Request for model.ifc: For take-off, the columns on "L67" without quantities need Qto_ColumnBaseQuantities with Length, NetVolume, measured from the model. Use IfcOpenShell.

First a look at what the model holds.

```python
import ifcopenshell
import ifcopenshell.util.element
import ifcopenshell.util.unit

model = ifcopenshell.open("model.ifc")
print(model.schema)
for unit_type in ("LENGTHUNIT", "AREAUNIT", "VOLUMEUNIT"):
    print(unit_type, ifcopenshell.util.unit.calculate_unit_scale(model, unit_type))
storey = next(s for s in model.by_type("IfcBuildingStorey") if s.Name == "L67")
columns = [e for e in ifcopenshell.util.element.get_decomposition(storey) if e.is_a("IfcColumn")]
for e in sorted(columns, key=lambda e: e.id()):
    print(e.id(), e.is_a(), e.Name, list(ifcopenshell.util.element.get_psets(e, qtos_only=True)), sep=" | ")
```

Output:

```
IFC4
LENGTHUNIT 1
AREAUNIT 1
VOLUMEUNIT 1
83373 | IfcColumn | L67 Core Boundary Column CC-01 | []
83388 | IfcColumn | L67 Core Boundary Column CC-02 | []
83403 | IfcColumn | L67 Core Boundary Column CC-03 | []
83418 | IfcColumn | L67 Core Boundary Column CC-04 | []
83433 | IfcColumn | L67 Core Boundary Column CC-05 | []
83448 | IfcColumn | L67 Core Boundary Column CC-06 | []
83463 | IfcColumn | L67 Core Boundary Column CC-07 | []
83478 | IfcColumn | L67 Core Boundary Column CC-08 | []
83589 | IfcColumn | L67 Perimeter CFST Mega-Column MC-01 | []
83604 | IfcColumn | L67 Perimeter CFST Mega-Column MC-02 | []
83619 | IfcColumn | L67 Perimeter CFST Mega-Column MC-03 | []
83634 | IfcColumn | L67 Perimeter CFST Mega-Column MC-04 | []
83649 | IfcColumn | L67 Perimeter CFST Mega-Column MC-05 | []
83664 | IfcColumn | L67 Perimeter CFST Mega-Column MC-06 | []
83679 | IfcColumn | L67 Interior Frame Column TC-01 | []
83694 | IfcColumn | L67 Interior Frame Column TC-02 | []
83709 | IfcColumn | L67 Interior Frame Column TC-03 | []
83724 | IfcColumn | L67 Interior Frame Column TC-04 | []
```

```python
import ifcopenshell
import ifcopenshell.api.pset
import ifcopenshell.geom
import ifcopenshell.util.element
import ifcopenshell.util.shape
import ifcopenshell.util.unit

model = ifcopenshell.open("model.ifc")
unit_scale = ifcopenshell.util.unit.calculate_unit_scale(model)
volume_scale = ifcopenshell.util.unit.calculate_unit_scale(model, "VOLUMEUNIT")
settings = ifcopenshell.geom.settings()

storey = next(s for s in model.by_type("IfcBuildingStorey") if s.Name == "L67")
columns = [e for e in ifcopenshell.util.element.get_decomposition(storey) if e.is_a("IfcColumn")]

for e in sorted(columns, key=lambda e: e.id()):
    if ifcopenshell.util.element.get_psets(e, qtos_only=True, should_inherit=False):
        continue
    # Geometry comes back in metres, in the element's own axes.
    shape = ifcopenshell.geom.create_shape(settings, e)
    values = {
        "Length": ifcopenshell.util.shape.get_z(shape.geometry) / unit_scale,
        "NetVolume": ifcopenshell.util.shape.get_volume(shape.geometry) / volume_scale,
    }
    qto = ifcopenshell.api.pset.add_qto(model, product=e, name="Qto_ColumnBaseQuantities")
    ifcopenshell.api.pset.edit_qto(model, qto=qto, properties=values)
    print(e.id(), {k: round(v, 3) for k, v in values.items()})

model.write("model_edited.ifc")
```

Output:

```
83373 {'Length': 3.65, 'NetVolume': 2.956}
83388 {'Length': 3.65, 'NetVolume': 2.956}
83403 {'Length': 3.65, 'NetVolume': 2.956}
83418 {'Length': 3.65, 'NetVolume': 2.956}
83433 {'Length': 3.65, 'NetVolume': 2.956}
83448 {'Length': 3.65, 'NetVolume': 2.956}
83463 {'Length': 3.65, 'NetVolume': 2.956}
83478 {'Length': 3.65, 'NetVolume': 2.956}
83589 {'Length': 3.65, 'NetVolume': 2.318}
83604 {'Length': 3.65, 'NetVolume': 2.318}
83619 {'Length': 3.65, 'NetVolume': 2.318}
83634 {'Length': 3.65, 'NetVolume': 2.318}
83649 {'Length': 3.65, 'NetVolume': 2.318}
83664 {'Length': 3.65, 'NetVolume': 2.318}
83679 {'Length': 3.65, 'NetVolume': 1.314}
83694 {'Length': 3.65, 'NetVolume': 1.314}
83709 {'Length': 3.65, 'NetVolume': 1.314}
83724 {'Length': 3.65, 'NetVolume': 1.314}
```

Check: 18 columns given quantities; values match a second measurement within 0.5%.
